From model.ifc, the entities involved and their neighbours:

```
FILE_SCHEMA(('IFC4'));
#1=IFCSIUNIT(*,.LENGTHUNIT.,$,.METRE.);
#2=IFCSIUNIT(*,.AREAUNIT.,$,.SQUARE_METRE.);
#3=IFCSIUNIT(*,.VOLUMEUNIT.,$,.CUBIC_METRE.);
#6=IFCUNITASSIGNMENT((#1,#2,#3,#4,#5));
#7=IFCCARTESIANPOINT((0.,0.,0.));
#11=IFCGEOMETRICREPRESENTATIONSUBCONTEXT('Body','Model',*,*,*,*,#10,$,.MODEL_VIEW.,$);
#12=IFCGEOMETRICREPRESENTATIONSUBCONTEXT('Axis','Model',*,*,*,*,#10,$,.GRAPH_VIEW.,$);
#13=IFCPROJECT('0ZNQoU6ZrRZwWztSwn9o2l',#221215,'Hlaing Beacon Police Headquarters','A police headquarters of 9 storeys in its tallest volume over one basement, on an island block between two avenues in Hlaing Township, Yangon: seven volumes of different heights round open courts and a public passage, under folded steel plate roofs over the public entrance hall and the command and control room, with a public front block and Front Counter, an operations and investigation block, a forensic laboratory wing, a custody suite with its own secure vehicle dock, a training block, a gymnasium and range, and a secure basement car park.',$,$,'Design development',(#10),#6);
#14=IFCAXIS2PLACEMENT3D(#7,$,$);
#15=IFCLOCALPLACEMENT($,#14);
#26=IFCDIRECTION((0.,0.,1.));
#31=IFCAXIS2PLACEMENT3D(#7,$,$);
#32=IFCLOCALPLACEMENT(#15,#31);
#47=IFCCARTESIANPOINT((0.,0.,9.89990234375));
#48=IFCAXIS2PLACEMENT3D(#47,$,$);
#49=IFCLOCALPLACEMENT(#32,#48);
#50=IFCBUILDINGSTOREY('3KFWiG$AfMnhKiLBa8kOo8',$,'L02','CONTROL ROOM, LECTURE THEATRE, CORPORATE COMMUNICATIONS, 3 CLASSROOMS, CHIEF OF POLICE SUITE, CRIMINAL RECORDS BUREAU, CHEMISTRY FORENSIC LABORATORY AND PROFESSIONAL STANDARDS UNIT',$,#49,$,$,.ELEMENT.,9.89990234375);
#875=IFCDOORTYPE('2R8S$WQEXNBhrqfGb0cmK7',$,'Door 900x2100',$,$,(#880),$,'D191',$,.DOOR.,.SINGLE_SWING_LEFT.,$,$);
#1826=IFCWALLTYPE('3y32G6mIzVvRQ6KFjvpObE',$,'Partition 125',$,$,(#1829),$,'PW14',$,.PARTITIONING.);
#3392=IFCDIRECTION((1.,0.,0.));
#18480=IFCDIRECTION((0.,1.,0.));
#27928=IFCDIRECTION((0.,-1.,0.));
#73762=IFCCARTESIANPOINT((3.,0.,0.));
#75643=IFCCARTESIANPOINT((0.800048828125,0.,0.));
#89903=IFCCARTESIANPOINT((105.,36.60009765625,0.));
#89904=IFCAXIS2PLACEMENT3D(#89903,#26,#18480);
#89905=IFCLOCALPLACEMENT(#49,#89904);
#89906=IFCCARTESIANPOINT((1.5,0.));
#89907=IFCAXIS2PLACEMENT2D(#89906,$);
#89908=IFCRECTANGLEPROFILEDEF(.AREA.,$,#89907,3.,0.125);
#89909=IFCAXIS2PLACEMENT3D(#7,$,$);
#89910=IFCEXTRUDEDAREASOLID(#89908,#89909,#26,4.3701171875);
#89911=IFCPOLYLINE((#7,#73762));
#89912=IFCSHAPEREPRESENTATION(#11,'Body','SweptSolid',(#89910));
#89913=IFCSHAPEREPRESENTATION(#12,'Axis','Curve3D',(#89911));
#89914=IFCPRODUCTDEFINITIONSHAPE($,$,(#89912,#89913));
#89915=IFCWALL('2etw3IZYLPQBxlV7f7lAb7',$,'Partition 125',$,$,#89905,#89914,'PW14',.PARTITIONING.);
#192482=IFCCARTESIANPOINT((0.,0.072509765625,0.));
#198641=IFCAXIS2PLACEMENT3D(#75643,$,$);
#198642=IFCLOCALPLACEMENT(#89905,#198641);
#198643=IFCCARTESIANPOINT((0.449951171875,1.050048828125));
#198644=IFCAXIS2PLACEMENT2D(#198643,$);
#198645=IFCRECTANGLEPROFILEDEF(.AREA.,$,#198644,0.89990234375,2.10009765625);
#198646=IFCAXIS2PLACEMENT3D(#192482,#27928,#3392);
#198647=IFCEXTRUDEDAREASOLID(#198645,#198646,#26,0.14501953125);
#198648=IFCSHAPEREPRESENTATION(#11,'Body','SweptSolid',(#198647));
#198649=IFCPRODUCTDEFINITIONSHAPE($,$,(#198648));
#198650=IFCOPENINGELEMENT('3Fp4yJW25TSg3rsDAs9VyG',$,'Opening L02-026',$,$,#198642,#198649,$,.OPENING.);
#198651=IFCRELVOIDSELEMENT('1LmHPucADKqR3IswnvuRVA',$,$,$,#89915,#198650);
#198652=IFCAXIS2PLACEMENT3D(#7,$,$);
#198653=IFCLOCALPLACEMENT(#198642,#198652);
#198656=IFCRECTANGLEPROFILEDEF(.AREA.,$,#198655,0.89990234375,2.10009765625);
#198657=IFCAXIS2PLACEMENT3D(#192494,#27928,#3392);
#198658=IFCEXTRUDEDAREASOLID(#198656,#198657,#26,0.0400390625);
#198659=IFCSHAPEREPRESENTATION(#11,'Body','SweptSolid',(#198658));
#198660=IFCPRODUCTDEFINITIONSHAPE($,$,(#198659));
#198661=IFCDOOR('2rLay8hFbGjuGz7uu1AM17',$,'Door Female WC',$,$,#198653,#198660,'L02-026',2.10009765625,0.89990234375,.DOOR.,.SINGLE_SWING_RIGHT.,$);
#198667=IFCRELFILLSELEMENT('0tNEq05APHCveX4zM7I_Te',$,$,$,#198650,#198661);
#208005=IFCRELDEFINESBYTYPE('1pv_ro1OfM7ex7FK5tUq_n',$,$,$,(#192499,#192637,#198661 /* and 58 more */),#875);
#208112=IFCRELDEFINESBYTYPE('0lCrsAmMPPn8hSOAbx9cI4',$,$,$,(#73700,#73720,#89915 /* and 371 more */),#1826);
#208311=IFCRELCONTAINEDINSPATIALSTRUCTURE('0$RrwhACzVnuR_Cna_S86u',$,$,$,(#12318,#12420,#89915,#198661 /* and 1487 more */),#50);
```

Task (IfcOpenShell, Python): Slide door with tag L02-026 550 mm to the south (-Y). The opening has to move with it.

```python
import ifcopenshell
import ifcopenshell.api.geometry
import ifcopenshell.util.placement

model = ifcopenshell.open("model.ifc")

door = model.by_guid("2rLay8hFbGjuGz7uu1AM17")
opening = door.FillsVoids[0].RelatingOpeningElement
wall = opening.VoidsElements[0].RelatingBuildingElement

wall_matrix = ifcopenshell.util.placement.get_local_placement(wall.ObjectPlacement)
shift = wall_matrix[:3, 0] * -0.55
before = ifcopenshell.util.placement.get_local_placement(door.ObjectPlacement)[:3, 3].copy()

# The door is placed relative to its opening, so it follows when the opening moves.
matrix = ifcopenshell.util.placement.get_local_placement(opening.ObjectPlacement)
matrix[:3, 3] += shift
ifcopenshell.api.geometry.edit_object_placement(
    model, product=opening, matrix=matrix, is_si=False, should_transform_children=True
)

after = ifcopenshell.util.placement.get_local_placement(door.ObjectPlacement)[:3, 3]
print("door moved by", (after - before).round(3) + 0.0)

model.write("model_rev.ifc")
```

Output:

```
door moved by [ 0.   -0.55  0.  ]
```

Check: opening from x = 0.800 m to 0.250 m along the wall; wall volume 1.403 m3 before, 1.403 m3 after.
